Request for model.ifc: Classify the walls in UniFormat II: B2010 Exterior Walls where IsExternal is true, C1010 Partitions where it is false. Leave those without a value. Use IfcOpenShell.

First a look at what the model holds.

```python
import ifcopenshell
import ifcopenshell.util.element

model = ifcopenshell.open("model.ifc")
print(model.schema)
print("classifications:", [c.Name for c in model.by_type("IfcClassification")])
values = [ifcopenshell.util.element.get_pset(e, "Pset_WallCommon", "IsExternal") for e in model.by_type("IfcWall")]
for value in (True, False, None):
    print("IsExternal", value, values.count(value))
```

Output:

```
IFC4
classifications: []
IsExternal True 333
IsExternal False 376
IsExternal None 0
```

```python
import ifcopenshell
import ifcopenshell.api.classification
import ifcopenshell.util.element

model = ifcopenshell.open("model.ifc")

system = ifcopenshell.api.classification.add_classification(model, classification="UniFormat II")

walls = model.by_type("IfcWall")
external = {e: ifcopenshell.util.element.get_pset(e, "Pset_WallCommon", "IsExternal") for e in walls}
for flag, code, name in ((True, "B2010", "Exterior Walls"), (False, "C1010", "Partitions")):
    products = [e for e in walls if external[e] is flag]
    ifcopenshell.api.classification.add_reference(
        model, products=products, classification=system, identification=code, name=name
    )
    print(code, len(products))

model.write("model_v2.ifc")
```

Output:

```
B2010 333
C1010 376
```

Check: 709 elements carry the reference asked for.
